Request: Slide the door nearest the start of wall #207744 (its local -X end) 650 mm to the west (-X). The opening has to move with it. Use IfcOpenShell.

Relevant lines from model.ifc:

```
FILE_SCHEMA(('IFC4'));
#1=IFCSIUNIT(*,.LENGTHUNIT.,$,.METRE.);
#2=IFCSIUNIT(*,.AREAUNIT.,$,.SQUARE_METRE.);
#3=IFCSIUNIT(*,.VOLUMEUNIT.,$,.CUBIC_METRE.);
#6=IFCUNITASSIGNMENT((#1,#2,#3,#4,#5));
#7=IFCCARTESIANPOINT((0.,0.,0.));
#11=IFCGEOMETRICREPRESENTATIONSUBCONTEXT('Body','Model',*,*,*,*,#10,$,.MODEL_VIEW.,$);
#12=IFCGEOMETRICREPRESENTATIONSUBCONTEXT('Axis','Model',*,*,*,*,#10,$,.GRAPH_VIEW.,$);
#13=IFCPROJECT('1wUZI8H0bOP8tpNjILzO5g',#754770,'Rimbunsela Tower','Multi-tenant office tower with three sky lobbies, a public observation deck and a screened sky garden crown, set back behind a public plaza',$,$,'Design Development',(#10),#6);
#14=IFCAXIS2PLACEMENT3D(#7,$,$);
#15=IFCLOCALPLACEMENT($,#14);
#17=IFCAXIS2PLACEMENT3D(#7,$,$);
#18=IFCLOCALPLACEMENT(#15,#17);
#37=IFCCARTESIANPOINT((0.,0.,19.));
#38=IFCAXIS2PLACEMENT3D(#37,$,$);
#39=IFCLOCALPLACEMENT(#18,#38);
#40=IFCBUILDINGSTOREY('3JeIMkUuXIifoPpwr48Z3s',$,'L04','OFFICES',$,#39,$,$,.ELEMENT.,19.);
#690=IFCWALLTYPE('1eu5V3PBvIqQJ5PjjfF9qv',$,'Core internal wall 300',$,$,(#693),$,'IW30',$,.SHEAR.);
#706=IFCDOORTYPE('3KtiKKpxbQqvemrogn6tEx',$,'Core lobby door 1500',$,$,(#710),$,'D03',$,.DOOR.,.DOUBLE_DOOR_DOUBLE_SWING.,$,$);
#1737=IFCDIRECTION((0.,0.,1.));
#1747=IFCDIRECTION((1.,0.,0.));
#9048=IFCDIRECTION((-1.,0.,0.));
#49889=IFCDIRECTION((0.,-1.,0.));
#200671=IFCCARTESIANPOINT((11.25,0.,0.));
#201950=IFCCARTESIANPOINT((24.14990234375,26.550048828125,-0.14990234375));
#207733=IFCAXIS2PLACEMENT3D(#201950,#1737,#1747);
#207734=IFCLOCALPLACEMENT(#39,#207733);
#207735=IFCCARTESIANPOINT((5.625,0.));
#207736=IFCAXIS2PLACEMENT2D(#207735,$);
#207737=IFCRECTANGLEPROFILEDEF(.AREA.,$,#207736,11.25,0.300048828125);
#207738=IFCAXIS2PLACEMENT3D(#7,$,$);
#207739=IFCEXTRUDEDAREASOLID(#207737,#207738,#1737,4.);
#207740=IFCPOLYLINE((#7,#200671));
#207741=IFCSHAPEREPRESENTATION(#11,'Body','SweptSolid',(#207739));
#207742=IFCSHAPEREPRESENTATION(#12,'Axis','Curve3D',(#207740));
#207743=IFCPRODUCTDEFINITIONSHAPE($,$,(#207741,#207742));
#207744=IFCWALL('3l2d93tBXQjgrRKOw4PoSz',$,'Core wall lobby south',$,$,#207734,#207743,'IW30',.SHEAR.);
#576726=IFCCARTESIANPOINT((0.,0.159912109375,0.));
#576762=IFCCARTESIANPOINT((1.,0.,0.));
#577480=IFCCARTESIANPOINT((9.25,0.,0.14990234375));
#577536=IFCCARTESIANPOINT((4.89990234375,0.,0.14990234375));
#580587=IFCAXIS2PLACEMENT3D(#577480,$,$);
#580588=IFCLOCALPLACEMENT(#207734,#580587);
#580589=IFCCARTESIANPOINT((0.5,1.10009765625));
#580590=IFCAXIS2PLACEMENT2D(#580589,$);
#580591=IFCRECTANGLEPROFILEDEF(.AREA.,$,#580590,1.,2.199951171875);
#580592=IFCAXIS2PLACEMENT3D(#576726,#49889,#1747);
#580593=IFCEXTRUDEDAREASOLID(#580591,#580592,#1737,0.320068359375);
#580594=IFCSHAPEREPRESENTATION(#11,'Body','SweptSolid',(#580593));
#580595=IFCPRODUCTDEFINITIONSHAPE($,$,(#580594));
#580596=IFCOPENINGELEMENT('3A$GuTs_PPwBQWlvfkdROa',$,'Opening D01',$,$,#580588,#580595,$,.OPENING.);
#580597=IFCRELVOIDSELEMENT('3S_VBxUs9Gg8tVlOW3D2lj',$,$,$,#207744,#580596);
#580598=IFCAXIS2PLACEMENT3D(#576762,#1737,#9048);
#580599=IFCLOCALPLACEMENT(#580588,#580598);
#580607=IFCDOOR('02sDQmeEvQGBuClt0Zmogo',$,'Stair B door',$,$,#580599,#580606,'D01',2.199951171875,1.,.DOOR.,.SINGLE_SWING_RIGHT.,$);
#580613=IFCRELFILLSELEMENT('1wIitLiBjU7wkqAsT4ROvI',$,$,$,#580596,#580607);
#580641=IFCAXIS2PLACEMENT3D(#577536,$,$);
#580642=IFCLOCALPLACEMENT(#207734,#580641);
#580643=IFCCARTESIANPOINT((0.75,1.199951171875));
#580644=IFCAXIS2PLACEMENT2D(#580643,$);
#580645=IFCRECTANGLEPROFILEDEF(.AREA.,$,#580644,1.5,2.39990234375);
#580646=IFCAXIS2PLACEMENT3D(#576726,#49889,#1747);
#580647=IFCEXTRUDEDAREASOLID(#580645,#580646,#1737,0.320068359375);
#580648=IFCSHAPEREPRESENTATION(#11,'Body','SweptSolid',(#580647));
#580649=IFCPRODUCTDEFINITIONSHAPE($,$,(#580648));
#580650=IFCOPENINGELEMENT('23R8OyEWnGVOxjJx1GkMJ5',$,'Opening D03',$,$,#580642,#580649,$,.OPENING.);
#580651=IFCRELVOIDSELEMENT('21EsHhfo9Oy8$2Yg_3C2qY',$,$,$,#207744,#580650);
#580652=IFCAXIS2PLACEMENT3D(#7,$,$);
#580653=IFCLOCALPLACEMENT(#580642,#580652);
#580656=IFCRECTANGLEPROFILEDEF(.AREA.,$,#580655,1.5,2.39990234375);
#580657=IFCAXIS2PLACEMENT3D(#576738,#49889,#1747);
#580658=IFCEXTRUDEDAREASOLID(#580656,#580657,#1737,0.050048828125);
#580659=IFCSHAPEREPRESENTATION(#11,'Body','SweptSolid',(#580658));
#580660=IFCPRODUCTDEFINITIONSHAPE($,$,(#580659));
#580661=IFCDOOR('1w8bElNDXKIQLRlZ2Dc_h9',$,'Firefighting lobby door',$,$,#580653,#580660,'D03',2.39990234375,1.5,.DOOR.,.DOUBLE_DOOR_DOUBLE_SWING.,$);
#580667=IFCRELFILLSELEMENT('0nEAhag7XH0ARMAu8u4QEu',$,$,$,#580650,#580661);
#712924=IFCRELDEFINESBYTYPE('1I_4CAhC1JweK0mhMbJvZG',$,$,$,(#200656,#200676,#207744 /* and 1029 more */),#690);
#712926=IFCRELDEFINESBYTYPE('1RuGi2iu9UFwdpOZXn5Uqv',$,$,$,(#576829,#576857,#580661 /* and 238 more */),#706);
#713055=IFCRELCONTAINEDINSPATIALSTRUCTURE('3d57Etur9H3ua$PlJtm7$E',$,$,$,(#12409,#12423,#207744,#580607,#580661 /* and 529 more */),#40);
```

```python
import ifcopenshell
import ifcopenshell.api.geometry
import ifcopenshell.util.placement
import ifcopenshell.util.unit

model = ifcopenshell.open("model.ifc")
unit_scale = ifcopenshell.util.unit.calculate_unit_scale(model)

door = model.by_id(580661)
opening = door.FillsVoids[0].RelatingOpeningElement
wall = opening.VoidsElements[0].RelatingBuildingElement

wall_matrix = ifcopenshell.util.placement.get_local_placement(wall.ObjectPlacement)
shift = wall_matrix[:3, 0] * -0.65 / unit_scale
before = ifcopenshell.util.placement.get_local_placement(door.ObjectPlacement)[:3, 3].copy()

# The door is placed relative to its opening, so it follows when the opening moves.
matrix = ifcopenshell.util.placement.get_local_placement(opening.ObjectPlacement)
matrix[:3, 3] += shift
ifcopenshell.api.geometry.edit_object_placement(
    model, product=opening, matrix=matrix, is_si=False, should_transform_children=True
)

after = ifcopenshell.util.placement.get_local_placement(door.ObjectPlacement)[:3, 3]
print("door moved by", (after - before).round(3) + 0.0)

model.write("model_v2.ifc")
```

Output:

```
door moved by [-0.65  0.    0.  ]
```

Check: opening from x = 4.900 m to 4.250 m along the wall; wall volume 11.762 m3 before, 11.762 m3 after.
